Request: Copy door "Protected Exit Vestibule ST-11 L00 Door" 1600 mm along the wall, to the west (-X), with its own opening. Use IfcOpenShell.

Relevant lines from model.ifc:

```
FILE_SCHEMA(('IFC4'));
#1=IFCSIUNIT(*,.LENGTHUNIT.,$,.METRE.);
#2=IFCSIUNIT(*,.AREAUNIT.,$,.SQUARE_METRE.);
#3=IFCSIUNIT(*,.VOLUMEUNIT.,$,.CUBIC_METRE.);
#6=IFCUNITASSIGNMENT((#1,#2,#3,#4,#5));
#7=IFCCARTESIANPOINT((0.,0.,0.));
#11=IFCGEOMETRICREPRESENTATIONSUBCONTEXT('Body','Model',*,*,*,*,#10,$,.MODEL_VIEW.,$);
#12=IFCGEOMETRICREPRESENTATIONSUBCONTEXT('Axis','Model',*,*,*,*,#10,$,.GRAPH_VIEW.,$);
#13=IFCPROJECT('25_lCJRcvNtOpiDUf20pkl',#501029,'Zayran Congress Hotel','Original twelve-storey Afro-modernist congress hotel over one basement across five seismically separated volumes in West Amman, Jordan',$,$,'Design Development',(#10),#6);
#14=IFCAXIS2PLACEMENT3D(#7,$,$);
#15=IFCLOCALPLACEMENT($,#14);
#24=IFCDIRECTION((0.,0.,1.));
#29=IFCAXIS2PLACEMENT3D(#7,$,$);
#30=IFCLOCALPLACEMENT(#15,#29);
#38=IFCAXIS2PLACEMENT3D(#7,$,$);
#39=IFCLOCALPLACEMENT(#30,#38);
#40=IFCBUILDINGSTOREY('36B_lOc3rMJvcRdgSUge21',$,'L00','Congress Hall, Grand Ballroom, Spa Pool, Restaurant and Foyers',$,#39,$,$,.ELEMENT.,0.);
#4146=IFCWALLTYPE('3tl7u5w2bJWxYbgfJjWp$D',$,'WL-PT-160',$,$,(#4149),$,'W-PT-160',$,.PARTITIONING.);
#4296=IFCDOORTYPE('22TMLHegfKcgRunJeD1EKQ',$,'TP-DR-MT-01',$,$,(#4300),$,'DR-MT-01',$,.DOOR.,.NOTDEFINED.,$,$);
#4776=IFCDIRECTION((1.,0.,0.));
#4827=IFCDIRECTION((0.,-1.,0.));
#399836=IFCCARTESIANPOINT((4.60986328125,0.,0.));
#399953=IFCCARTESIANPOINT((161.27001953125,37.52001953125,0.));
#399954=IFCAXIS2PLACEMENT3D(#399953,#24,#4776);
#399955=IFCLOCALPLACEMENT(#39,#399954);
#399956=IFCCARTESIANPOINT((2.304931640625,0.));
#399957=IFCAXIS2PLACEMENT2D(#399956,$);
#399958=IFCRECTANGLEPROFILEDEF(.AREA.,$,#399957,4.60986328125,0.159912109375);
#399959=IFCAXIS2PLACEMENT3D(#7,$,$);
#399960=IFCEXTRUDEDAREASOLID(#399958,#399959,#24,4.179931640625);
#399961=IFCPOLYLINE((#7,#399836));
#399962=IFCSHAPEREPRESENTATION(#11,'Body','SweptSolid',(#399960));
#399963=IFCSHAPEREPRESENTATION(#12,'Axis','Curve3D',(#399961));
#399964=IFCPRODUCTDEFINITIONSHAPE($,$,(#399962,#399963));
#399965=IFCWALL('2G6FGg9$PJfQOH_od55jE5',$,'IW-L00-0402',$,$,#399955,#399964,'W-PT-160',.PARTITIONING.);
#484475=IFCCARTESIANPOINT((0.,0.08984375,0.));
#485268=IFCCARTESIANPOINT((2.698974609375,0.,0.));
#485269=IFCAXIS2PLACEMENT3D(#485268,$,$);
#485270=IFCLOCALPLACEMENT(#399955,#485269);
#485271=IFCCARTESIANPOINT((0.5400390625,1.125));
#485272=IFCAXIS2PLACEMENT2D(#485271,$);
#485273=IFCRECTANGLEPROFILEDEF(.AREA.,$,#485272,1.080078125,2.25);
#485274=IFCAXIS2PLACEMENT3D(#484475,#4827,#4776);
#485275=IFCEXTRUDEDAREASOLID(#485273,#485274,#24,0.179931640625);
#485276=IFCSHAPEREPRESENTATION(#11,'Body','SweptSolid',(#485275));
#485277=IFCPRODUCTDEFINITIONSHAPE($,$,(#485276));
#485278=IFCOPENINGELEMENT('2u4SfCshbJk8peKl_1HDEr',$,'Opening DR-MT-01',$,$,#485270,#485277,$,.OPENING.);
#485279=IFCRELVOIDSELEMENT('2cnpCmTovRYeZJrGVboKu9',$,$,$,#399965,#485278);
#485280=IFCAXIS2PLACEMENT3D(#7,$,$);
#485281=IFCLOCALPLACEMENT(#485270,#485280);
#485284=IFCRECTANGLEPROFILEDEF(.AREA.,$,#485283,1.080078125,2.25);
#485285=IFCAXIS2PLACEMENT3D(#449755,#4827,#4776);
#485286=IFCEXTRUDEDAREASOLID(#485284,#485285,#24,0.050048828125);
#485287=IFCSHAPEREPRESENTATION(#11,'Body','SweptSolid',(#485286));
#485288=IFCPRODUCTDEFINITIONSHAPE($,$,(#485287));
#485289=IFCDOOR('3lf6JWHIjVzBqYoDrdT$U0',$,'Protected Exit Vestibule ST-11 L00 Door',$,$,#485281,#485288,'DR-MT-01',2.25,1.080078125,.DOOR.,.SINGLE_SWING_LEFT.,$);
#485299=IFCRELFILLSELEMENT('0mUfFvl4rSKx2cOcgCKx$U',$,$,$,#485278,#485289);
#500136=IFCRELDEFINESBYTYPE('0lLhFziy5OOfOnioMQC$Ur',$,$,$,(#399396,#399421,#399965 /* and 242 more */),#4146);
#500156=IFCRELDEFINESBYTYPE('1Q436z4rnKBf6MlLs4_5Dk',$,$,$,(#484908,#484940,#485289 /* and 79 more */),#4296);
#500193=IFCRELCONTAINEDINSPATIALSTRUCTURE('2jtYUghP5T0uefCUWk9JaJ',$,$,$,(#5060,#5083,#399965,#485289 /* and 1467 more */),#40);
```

```python
import ifcopenshell
import ifcopenshell.api.feature
import ifcopenshell.api.geometry
import ifcopenshell.api.root
import ifcopenshell.geom
import ifcopenshell.util.element
import ifcopenshell.util.placement
import ifcopenshell.util.shape

model = ifcopenshell.open("model.ifc")
settings = ifcopenshell.geom.settings()


def volume(element):
    """Net volume in cubic metres, openings subtracted."""
    shape = ifcopenshell.geom.create_shape(settings, element)
    return ifcopenshell.util.shape.get_volume(shape.geometry)


door = model.by_guid("3lf6JWHIjVzBqYoDrdT$U0")
opening = door.FillsVoids[0].RelatingOpeningElement
wall = opening.VoidsElements[0].RelatingBuildingElement
before = volume(wall)
shift = ifcopenshell.util.placement.get_local_placement(wall.ObjectPlacement)[:3, 0] * -1.6

# copy_class copies the void relationship, type, container and properties, but no geometry.
new_opening = ifcopenshell.api.root.copy_class(model, product=opening)
new_opening.Representation = ifcopenshell.util.element.copy_deep(
    model, opening.Representation, exclude=["IfcGeometricRepresentationContext", "IfcRepresentationMap"]
)
new_door = ifcopenshell.api.root.copy_class(model, product=door)
new_door.Representation = ifcopenshell.util.element.copy_deep(
    model, door.Representation, exclude=["IfcGeometricRepresentationContext", "IfcRepresentationMap"]
)
new_door.Tag = None
ifcopenshell.api.feature.add_filling(model, opening=new_opening, element=new_door)

for old, new in ((opening, new_opening), (door, new_door)):
    matrix = ifcopenshell.util.placement.get_local_placement(old.ObjectPlacement)
    matrix[:3, 3] += shift
    ifcopenshell.api.geometry.edit_object_placement(model, product=new, matrix=matrix, is_si=False)

after = volume(wall)

print(f"wall volume {before:.3f} -> {after:.3f} m3")

model.write("model_v2.ifc")
```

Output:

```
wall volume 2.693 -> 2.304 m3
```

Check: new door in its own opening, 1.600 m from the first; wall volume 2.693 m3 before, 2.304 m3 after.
